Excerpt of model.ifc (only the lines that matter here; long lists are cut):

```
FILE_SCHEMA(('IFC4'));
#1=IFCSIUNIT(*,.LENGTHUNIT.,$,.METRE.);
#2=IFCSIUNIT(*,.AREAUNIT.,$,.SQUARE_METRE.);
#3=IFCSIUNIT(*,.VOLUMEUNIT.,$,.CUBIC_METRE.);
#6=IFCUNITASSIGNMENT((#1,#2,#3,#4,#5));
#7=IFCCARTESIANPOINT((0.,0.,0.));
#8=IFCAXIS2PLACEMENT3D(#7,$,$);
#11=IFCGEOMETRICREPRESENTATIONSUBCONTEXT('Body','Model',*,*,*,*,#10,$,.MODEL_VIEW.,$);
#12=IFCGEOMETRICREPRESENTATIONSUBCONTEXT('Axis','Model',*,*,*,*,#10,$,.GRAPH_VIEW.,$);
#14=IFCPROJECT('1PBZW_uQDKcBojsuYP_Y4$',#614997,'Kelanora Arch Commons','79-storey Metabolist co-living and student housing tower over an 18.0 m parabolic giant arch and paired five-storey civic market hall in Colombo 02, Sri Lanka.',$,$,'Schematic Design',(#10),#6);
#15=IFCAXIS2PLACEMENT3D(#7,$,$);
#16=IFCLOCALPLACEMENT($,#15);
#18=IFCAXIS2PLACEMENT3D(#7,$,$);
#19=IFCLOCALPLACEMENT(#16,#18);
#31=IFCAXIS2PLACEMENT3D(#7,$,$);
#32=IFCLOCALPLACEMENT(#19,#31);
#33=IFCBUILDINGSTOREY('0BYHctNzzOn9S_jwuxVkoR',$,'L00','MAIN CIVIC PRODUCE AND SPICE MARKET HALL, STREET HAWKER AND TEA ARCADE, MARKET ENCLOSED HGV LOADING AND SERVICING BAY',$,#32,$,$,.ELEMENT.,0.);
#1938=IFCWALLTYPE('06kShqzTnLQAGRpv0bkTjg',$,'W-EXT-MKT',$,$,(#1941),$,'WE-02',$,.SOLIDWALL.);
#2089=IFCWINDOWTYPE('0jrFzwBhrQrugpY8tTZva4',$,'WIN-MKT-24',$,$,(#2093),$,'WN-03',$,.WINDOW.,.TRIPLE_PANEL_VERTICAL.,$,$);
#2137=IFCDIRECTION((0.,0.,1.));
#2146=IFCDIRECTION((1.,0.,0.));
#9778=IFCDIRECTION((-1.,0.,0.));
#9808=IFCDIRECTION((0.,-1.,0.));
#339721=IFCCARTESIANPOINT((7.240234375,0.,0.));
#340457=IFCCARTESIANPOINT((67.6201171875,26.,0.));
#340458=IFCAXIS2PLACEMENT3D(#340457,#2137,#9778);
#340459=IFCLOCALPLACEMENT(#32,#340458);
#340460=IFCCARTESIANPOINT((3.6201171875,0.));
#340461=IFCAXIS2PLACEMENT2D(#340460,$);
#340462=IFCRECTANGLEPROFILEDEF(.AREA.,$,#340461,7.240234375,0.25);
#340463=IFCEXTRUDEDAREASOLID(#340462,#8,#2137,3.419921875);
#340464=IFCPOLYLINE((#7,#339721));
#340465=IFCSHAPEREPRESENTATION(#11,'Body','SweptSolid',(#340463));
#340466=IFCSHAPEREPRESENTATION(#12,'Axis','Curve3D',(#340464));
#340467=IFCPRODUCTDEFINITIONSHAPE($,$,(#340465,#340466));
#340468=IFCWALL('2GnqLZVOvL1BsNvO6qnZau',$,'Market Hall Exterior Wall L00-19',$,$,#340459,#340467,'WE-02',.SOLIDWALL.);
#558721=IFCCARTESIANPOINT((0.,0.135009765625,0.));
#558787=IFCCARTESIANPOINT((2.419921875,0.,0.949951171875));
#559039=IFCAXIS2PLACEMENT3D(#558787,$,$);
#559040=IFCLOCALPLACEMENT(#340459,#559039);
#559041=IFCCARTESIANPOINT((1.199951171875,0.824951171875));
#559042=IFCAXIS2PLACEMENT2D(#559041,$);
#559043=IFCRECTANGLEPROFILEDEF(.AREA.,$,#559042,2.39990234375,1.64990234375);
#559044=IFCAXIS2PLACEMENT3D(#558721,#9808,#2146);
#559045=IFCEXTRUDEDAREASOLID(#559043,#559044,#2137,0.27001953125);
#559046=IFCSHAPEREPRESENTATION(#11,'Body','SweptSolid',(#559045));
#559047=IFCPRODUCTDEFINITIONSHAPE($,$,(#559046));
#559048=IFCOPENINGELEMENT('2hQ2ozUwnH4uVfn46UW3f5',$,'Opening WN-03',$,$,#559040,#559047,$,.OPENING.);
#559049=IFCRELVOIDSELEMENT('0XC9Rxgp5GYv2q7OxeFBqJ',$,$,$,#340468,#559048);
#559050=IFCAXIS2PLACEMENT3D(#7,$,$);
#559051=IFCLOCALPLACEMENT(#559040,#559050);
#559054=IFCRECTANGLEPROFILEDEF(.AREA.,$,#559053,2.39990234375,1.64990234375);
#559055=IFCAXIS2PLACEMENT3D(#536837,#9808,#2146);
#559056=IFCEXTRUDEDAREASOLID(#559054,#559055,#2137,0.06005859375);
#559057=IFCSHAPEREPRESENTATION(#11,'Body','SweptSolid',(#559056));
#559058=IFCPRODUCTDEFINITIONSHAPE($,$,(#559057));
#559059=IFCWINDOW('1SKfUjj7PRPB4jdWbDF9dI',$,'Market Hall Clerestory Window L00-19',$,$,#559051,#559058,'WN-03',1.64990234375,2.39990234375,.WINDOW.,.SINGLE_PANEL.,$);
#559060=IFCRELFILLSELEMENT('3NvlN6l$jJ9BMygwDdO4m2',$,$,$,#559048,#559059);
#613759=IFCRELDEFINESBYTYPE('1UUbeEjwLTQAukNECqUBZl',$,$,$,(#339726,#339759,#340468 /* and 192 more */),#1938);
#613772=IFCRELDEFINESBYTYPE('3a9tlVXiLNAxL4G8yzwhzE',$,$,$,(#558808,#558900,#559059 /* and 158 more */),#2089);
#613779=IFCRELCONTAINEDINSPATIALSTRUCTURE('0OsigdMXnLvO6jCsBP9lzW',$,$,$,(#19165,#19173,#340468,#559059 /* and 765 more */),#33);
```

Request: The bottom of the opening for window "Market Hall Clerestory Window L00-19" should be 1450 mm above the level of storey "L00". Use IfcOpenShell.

```python
import numpy as np
import ifcopenshell
import ifcopenshell.api.geometry
import ifcopenshell.geom
import ifcopenshell.util.element
import ifcopenshell.util.placement
import ifcopenshell.util.shape
import ifcopenshell.util.unit

model = ifcopenshell.open("model.ifc")
unit_scale = ifcopenshell.util.unit.calculate_unit_scale(model)

window = model.by_guid("1SKfUjj7PRPB4jdWbDF9dI")
opening = window.FillsVoids[0].RelatingOpeningElement
storey = ifcopenshell.util.element.get_container(window, ifc_class="IfcBuildingStorey")
level = ifcopenshell.util.placement.get_local_placement(storey.ObjectPlacement)[2, 3]

# The opening's origin need not be at the sill, so measure its lowest point.
shape = ifcopenshell.geom.create_shape(ifcopenshell.geom.settings(), opening)
bottom = ifcopenshell.util.shape.get_shape_bottom_elevation(shape, shape.geometry) / unit_scale
dz = level + 1.45 - bottom

shift = np.array([0.0, 0.0, dz])
# The window is placed relative to its opening, so it follows when the opening moves.
matrix = ifcopenshell.util.placement.get_local_placement(opening.ObjectPlacement)
matrix[:3, 3] += shift
ifcopenshell.api.geometry.edit_object_placement(
    model, product=opening, matrix=matrix, is_si=False, should_transform_children=True
)

print(f"moved by {dz * unit_scale:+.3f} m")

model.write("model_v2.ifc")
```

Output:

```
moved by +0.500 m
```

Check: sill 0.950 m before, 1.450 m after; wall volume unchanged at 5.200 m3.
